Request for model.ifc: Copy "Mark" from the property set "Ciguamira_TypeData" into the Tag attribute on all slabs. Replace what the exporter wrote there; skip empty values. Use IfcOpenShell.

First a look at what the model holds.

```python
import ifcopenshell
import ifcopenshell.util.element

model = ifcopenshell.open("model.ifc")
print(model.schema)
slabs = model.by_type("IfcSlab")
print(len(slabs), "slabs")
for e in slabs[:8]:
    source = ifcopenshell.util.element.get_pset(e, "Ciguamira_TypeData", "Mark")
    target = e.Tag
    print(e.id(), repr(source), repr(target), sep=" | ")
```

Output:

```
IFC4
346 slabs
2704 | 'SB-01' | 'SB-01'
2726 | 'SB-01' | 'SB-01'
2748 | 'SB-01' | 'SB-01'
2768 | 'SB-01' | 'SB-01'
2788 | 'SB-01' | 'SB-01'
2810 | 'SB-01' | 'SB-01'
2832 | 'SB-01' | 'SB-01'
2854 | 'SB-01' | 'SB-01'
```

```python
import ifcopenshell
import ifcopenshell.util.element

model = ifcopenshell.open("model.ifc")

count = 0
for e in model.by_type("IfcSlab"):
    value = ifcopenshell.util.element.get_pset(e, "Ciguamira_TypeData", "Mark")
    current = e.Tag
    if not value or not value.strip() or current == value:
        continue
    e.Tag = value
    count += 1

print(count, "slabs updated")

model.write("model_rev.ifc")
```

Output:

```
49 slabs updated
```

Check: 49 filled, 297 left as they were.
